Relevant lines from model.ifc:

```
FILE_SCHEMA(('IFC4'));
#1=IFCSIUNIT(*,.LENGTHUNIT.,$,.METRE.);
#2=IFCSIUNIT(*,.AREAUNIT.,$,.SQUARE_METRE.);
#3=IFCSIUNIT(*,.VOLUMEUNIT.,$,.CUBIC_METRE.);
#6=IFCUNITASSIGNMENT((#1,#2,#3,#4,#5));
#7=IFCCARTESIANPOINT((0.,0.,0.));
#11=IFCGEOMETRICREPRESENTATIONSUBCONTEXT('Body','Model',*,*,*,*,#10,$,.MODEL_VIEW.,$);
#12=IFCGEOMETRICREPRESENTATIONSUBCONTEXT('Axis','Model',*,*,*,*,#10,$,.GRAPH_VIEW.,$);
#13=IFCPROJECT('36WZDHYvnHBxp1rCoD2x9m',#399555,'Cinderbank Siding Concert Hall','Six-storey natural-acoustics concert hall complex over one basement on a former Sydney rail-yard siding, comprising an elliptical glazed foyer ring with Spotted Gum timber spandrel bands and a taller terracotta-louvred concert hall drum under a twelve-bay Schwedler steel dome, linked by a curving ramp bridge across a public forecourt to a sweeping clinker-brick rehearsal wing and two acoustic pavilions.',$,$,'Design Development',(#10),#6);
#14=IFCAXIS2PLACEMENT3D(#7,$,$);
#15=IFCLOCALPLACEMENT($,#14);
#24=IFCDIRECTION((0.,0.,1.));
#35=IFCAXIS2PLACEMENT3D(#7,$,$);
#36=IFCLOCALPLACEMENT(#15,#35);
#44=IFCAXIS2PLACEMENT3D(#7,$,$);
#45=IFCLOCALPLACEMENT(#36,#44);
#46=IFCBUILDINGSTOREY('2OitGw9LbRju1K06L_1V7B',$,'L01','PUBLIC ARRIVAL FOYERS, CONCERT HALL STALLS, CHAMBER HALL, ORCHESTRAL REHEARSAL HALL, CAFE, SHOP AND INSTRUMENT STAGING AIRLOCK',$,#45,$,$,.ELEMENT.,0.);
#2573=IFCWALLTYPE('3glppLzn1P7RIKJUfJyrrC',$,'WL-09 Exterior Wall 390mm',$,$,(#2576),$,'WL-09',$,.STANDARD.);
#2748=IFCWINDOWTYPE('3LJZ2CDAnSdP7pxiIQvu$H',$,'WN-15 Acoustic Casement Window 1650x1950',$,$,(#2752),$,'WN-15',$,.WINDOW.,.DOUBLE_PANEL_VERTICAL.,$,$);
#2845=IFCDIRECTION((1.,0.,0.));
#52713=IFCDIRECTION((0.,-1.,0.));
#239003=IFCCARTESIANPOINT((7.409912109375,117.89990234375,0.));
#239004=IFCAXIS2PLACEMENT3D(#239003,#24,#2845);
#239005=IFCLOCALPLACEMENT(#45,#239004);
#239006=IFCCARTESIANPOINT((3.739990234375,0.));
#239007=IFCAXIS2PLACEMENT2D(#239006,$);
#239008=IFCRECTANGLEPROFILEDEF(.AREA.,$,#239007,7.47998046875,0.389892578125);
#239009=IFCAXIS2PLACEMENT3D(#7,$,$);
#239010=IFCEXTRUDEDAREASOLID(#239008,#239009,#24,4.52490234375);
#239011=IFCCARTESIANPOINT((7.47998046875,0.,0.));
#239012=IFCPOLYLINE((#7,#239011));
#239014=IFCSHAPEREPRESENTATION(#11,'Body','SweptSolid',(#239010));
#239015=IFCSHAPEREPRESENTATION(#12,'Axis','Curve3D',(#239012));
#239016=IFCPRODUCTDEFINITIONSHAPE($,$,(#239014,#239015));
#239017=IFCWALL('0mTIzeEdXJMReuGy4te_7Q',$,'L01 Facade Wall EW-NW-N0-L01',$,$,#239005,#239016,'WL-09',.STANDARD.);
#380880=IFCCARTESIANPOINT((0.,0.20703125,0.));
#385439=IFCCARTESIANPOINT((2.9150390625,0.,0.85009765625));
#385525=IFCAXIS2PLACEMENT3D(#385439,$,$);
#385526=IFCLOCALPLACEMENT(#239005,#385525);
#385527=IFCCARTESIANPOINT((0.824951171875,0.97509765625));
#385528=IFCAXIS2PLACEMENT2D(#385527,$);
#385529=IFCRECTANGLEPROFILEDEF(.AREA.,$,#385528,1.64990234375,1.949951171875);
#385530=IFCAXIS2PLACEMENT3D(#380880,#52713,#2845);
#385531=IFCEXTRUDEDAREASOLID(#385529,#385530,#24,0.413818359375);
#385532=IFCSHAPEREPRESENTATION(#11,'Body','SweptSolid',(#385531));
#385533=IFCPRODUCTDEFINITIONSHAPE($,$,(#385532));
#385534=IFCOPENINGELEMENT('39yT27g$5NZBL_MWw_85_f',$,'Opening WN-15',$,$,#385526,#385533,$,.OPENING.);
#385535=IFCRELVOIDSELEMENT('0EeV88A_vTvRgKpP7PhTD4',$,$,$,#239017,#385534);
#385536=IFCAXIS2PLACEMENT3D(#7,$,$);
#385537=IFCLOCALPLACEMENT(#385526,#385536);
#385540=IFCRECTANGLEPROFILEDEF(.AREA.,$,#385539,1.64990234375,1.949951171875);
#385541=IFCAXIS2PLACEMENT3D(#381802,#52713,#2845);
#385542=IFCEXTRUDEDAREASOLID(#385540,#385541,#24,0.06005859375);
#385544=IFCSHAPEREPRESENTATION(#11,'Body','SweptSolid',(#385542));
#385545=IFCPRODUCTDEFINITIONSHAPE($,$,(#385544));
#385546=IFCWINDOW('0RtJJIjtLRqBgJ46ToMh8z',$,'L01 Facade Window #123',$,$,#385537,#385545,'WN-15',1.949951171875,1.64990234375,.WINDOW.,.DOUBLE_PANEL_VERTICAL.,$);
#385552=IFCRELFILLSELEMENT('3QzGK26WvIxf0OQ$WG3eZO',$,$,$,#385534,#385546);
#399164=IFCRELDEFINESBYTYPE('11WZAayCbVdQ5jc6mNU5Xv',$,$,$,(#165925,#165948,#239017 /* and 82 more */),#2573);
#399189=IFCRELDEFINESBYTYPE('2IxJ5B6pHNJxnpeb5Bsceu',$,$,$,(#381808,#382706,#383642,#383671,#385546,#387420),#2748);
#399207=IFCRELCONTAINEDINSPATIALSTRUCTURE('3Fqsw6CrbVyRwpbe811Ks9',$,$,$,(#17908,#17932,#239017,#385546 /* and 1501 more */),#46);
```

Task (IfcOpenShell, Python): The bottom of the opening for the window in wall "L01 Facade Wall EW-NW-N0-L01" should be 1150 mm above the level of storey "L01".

```python
import numpy as np
import ifcopenshell
import ifcopenshell.api.geometry
import ifcopenshell.geom
import ifcopenshell.util.element
import ifcopenshell.util.placement
import ifcopenshell.util.shape
import ifcopenshell.util.unit

model = ifcopenshell.open("model.ifc")
unit_scale = ifcopenshell.util.unit.calculate_unit_scale(model)

window = model.by_id(385546)
opening = window.FillsVoids[0].RelatingOpeningElement
storey = ifcopenshell.util.element.get_container(window, ifc_class="IfcBuildingStorey")
level = ifcopenshell.util.placement.get_local_placement(storey.ObjectPlacement)[2, 3]

# The opening's origin need not be at the sill, so measure its lowest point.
shape = ifcopenshell.geom.create_shape(ifcopenshell.geom.settings(), opening)
bottom = ifcopenshell.util.shape.get_shape_bottom_elevation(shape, shape.geometry) / unit_scale
dz = level + 1.15 / unit_scale - bottom

shift = np.array([0.0, 0.0, dz])
# The window is placed relative to its opening, so it follows when the opening moves.
matrix = ifcopenshell.util.placement.get_local_placement(opening.ObjectPlacement)
matrix[:3, 3] += shift
ifcopenshell.api.geometry.edit_object_placement(
    model, product=opening, matrix=matrix, is_si=False, should_transform_children=True
)

print(f"moved by {dz * unit_scale:+.3f} m")

model.write("model-out.ifc")
```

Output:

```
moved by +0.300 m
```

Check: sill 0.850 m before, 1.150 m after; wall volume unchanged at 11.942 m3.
